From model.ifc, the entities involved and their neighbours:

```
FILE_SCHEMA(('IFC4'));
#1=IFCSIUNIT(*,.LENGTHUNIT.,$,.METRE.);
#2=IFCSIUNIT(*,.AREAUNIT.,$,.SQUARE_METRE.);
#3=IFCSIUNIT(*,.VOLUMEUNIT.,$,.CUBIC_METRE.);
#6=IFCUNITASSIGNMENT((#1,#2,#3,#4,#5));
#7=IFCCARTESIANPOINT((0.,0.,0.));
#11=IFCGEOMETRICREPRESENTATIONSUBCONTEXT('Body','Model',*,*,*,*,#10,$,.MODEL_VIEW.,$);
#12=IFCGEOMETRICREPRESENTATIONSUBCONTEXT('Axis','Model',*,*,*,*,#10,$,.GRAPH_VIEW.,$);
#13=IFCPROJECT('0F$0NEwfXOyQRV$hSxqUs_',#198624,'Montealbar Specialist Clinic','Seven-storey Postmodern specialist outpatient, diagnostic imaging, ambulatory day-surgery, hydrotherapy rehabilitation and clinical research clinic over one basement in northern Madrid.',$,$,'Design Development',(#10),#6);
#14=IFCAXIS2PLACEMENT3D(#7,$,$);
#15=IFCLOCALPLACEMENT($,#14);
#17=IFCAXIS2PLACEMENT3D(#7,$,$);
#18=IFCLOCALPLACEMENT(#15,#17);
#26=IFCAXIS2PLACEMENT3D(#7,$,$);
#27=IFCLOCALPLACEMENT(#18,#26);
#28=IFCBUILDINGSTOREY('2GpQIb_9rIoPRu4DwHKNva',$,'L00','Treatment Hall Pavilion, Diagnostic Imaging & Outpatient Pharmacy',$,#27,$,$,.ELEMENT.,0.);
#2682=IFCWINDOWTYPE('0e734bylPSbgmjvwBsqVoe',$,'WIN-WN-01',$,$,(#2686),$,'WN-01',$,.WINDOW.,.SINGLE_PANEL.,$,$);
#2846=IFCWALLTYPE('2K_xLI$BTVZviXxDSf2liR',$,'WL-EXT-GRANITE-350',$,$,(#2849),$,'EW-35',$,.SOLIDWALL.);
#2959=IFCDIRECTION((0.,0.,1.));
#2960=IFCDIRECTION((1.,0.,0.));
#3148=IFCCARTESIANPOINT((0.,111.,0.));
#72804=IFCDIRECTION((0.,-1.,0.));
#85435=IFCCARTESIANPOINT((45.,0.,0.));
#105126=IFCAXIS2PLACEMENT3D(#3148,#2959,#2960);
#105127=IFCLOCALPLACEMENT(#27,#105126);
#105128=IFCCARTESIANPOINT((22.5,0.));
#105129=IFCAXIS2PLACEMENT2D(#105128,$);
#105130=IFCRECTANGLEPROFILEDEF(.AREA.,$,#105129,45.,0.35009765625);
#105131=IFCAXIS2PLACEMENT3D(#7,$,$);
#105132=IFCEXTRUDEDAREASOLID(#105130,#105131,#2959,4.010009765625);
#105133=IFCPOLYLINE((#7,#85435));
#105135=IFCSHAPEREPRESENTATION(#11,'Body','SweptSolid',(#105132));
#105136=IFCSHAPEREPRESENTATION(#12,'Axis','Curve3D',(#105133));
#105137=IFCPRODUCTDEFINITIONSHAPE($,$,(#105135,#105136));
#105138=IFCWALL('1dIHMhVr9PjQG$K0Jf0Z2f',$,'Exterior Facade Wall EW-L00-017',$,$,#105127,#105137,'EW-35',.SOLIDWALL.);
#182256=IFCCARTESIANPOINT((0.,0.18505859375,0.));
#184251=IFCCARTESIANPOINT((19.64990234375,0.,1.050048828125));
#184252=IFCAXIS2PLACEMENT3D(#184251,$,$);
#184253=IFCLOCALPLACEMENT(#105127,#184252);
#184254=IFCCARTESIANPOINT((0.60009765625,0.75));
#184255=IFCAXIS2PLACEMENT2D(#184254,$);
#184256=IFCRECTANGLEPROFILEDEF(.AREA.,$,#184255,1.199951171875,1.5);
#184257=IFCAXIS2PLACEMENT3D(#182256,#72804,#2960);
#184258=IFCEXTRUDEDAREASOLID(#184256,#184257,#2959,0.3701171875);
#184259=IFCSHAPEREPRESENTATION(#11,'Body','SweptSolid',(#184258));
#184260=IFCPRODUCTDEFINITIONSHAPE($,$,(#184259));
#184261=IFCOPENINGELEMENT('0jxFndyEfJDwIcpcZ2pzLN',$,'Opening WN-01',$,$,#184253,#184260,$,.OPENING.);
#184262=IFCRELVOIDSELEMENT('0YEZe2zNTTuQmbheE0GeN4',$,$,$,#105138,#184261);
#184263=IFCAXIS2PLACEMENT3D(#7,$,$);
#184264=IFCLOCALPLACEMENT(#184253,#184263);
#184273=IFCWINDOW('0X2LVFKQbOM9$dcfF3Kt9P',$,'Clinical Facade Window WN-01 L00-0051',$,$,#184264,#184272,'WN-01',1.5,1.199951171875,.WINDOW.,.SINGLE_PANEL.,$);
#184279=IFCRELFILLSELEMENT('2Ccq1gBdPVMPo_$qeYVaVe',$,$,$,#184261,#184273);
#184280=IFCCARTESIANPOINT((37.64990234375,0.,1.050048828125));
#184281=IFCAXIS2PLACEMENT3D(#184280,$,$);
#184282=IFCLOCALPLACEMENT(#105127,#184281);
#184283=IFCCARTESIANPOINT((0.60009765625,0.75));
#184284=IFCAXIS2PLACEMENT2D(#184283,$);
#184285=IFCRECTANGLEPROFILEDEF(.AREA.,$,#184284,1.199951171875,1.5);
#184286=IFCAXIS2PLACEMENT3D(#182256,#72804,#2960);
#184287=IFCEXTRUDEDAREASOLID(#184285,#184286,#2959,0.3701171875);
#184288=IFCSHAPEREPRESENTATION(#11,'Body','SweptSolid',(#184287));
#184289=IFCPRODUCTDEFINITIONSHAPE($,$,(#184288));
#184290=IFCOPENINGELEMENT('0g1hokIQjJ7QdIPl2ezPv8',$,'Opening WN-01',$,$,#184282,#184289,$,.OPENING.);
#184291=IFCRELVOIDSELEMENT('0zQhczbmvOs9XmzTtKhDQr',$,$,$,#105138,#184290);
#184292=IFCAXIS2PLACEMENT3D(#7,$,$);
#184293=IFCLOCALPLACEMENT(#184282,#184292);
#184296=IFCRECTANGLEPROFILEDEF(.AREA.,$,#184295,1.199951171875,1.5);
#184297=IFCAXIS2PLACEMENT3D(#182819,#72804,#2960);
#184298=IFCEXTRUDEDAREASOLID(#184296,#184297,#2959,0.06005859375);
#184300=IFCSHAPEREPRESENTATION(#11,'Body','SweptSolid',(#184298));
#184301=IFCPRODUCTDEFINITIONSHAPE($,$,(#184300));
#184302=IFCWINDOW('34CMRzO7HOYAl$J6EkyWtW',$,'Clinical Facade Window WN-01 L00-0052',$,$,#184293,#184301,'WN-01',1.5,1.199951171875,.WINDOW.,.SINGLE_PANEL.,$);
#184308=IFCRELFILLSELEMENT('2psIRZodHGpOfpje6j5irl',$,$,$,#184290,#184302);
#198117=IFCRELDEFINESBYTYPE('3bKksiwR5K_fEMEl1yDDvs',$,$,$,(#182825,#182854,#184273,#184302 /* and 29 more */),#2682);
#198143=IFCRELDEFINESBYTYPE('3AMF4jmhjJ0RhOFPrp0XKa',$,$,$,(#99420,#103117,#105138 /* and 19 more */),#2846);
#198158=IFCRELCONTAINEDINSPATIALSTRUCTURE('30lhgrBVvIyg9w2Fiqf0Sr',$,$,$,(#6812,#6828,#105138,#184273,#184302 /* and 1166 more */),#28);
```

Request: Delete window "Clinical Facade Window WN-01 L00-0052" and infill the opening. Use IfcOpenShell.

```python
import ifcopenshell
import ifcopenshell.api.feature
import ifcopenshell.api.root
import ifcopenshell.geom
import ifcopenshell.util.shape

model = ifcopenshell.open("model.ifc")
settings = ifcopenshell.geom.settings()


def volume(element):
    """Net volume in cubic metres, openings subtracted."""
    shape = ifcopenshell.geom.create_shape(settings, element)
    return ifcopenshell.util.shape.get_volume(shape.geometry)


window = model.by_guid("34CMRzO7HOYAl$J6EkyWtW")
opening = window.FillsVoids[0].RelatingOpeningElement
wall = opening.VoidsElements[0].RelatingBuildingElement
before = volume(wall)

ifcopenshell.api.root.remove_product(model, product=window)
ifcopenshell.api.feature.remove_feature(model, feature=opening)

after = volume(wall)

print(f"wall volume {before:.3f} -> {after:.3f} m3")

model.write("model_v2.ifc")
```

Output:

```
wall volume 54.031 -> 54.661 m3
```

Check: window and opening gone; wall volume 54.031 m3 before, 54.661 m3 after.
